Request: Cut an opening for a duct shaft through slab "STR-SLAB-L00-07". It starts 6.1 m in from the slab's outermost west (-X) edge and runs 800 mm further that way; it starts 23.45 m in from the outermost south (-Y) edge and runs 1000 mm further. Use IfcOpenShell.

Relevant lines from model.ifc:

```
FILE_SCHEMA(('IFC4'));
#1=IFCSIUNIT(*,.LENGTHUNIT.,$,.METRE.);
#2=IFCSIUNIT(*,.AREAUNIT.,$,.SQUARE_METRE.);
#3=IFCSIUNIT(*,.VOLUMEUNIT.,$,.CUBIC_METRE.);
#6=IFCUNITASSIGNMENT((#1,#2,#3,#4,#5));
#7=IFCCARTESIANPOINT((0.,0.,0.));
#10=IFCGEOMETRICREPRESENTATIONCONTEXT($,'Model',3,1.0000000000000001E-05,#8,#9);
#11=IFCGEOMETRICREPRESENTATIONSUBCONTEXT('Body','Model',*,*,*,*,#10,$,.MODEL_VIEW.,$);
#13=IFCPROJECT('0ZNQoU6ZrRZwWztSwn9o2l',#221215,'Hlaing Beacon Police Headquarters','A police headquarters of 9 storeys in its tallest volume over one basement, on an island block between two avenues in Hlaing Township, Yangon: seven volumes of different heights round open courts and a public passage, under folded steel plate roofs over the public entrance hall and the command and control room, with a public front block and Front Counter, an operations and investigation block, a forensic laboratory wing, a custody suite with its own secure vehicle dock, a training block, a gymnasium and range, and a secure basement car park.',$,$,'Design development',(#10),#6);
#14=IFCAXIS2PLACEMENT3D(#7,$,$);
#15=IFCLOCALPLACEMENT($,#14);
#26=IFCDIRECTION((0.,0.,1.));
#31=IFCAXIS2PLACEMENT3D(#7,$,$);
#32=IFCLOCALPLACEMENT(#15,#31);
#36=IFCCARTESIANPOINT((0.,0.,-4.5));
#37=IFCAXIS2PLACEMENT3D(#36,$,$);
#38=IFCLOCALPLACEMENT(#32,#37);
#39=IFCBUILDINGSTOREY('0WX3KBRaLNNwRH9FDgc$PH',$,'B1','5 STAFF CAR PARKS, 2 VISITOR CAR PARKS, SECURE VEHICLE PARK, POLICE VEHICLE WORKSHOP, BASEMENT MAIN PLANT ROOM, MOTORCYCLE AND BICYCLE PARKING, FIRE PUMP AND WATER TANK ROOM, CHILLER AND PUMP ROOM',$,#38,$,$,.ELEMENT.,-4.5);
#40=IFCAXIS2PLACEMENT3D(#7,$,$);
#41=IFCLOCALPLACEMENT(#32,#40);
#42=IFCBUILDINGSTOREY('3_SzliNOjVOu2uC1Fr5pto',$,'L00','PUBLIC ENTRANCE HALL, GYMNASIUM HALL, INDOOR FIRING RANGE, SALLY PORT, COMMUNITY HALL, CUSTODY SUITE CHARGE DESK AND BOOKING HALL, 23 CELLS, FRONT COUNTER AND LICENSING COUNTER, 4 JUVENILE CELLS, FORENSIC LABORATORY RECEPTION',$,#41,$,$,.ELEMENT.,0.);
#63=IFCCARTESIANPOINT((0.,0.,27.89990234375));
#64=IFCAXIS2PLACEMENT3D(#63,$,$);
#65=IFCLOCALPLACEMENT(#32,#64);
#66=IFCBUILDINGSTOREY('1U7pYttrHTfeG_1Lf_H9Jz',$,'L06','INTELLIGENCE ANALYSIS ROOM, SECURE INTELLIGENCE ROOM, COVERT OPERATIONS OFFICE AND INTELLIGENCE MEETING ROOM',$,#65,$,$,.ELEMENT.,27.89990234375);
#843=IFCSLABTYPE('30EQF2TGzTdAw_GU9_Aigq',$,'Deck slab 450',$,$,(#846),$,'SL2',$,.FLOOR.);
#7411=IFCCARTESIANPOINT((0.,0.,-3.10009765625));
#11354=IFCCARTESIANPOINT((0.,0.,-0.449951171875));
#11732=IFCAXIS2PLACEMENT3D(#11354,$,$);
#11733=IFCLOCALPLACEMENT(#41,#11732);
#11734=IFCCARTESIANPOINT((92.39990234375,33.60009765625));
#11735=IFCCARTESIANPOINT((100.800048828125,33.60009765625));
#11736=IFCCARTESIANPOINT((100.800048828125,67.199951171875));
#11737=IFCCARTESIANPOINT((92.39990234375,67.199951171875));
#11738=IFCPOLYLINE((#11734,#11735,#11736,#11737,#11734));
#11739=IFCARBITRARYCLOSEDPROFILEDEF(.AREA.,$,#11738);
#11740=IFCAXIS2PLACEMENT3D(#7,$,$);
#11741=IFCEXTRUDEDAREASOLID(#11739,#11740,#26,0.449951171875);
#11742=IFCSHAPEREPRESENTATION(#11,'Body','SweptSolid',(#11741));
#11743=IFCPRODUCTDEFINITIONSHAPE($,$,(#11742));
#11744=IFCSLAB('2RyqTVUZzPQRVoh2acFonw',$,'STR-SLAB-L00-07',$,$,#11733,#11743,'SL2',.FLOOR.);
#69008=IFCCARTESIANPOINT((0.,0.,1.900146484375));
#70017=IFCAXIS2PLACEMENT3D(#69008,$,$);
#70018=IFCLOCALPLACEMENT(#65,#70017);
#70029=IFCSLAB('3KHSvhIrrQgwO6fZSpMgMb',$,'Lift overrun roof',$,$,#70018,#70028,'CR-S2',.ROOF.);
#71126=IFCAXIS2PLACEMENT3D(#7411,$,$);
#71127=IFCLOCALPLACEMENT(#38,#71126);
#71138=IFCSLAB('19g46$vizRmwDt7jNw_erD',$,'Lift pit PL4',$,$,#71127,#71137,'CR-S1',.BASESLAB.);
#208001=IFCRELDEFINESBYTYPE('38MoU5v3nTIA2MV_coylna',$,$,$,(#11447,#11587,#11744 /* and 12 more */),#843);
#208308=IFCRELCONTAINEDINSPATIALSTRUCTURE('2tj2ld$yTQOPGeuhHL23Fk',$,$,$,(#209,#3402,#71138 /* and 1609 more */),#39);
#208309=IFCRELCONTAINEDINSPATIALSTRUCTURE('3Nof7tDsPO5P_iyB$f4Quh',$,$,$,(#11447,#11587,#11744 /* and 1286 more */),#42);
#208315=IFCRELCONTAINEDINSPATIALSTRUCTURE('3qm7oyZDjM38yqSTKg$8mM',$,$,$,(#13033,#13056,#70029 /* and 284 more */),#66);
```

```python
import numpy as np
import ifcopenshell
import ifcopenshell.api.feature
import ifcopenshell.api.geometry
import ifcopenshell.api.root
import ifcopenshell.geom
import ifcopenshell.util.placement
import ifcopenshell.util.representation
import ifcopenshell.util.shape
import ifcopenshell.util.unit

model = ifcopenshell.open("model.ifc")
unit_scale = ifcopenshell.util.unit.calculate_unit_scale(model)
settings = ifcopenshell.geom.settings()


def volume(element):
    """Net volume in cubic metres, openings subtracted."""
    shape = ifcopenshell.geom.create_shape(settings, element)
    return ifcopenshell.util.shape.get_volume(shape.geometry)


slab = model.by_id(11744)
before = volume(slab)

# Extent in the slab's own axes, in metres. The edges named are its -X and -Y sides.
slab_shape = ifcopenshell.geom.create_shape(settings, slab)
vertices = ifcopenshell.util.shape.get_vertices(slab_shape.geometry)
x_min, y_min, bottom = vertices.min(axis=0)
top = vertices[:, 2].max()

opening = ifcopenshell.api.root.create_entity(model, ifc_class="IfcOpeningElement", name="Duct shaft opening", predefined_type="OPENING")
context = ifcopenshell.util.representation.get_context(model, "Model", "Body", "MODEL_VIEW")
width, depth = 0.8, 1
outline = [(0.0, 0.0), (width, 0.0), (width, depth), (0.0, depth), (0.0, 0.0)]
# Overshoot both faces by 50 mm so the cut is clean.
shape = ifcopenshell.api.geometry.add_slab_representation(
    model, context=context, depth=top - bottom + 0.1, polyline=outline
)
ifcopenshell.api.geometry.assign_representation(model, product=opening, representation=shape)

matrix = ifcopenshell.util.placement.get_local_placement(slab.ObjectPlacement)
matrix[:, 3] = matrix @ np.append(np.array([x_min + 6.1, y_min + 23.45, bottom - 0.05]) / unit_scale, 1.0)
ifcopenshell.api.geometry.edit_object_placement(model, product=opening, matrix=matrix, is_si=False)
ifcopenshell.api.feature.add_feature(model, feature=opening, element=slab)

after = volume(slab)

print(f"slab volume {before:.3f} -> {after:.3f} m3")

model.write("model_v2.ifc")
```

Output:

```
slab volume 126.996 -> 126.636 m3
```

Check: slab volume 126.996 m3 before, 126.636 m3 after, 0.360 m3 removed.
